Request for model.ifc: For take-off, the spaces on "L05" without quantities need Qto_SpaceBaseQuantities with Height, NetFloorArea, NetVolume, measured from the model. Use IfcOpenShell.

First a look at what the model holds.

```python
import ifcopenshell
import ifcopenshell.util.element
import ifcopenshell.util.unit

model = ifcopenshell.open("model.ifc")
print(model.schema)
for unit_type in ("LENGTHUNIT", "AREAUNIT", "VOLUMEUNIT"):
    print(unit_type, ifcopenshell.util.unit.calculate_unit_scale(model, unit_type))
storey = next(s for s in model.by_type("IfcBuildingStorey") if s.Name == "L05")
spaces = [e for e in ifcopenshell.util.element.get_decomposition(storey) if e.is_a("IfcSpace")]
for e in sorted(spaces, key=lambda e: e.id()):
    print(e.id(), e.is_a(), e.Name, list(ifcopenshell.util.element.get_psets(e, qtos_only=True)), sep=" | ")
```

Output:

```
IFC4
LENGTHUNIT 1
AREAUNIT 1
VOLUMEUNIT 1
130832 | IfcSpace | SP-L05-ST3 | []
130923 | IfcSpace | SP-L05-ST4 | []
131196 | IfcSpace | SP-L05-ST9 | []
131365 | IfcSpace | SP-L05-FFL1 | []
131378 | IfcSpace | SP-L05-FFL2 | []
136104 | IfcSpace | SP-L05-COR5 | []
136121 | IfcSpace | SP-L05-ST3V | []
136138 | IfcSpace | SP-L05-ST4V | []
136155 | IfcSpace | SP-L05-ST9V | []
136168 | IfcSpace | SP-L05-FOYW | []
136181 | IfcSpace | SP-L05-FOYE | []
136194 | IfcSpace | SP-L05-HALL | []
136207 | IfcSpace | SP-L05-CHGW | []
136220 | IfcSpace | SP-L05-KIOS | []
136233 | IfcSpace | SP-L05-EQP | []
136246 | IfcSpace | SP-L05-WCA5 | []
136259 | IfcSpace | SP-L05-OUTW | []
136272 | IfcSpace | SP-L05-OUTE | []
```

```python
import ifcopenshell
import ifcopenshell.api.pset
import ifcopenshell.geom
import ifcopenshell.util.element
import ifcopenshell.util.shape
import ifcopenshell.util.unit

model = ifcopenshell.open("model.ifc")
unit_scale = ifcopenshell.util.unit.calculate_unit_scale(model)
area_scale = ifcopenshell.util.unit.calculate_unit_scale(model, "AREAUNIT")
volume_scale = ifcopenshell.util.unit.calculate_unit_scale(model, "VOLUMEUNIT")
settings = ifcopenshell.geom.settings()

storey = next(s for s in model.by_type("IfcBuildingStorey") if s.Name == "L05")
spaces = [e for e in ifcopenshell.util.element.get_decomposition(storey) if e.is_a("IfcSpace")]

for e in sorted(spaces, key=lambda e: e.id()):
    if ifcopenshell.util.element.get_psets(e, qtos_only=True, should_inherit=False):
        continue
    # Geometry comes back in metres, in the element's own axes.
    shape = ifcopenshell.geom.create_shape(settings, e)
    values = {
        "Height": ifcopenshell.util.shape.get_z(shape.geometry) / unit_scale,
        "NetFloorArea": ifcopenshell.util.shape.get_footprint_area(shape.geometry) / area_scale,
        "NetVolume": ifcopenshell.util.shape.get_volume(shape.geometry) / volume_scale,
    }
    qto = ifcopenshell.api.pset.add_qto(model, product=e, name="Qto_SpaceBaseQuantities")
    ifcopenshell.api.pset.edit_qto(model, qto=qto, properties=values)
    print(e.id(), {k: round(v, 3) for k, v in values.items()})

model.write("model_edited.ifc")
```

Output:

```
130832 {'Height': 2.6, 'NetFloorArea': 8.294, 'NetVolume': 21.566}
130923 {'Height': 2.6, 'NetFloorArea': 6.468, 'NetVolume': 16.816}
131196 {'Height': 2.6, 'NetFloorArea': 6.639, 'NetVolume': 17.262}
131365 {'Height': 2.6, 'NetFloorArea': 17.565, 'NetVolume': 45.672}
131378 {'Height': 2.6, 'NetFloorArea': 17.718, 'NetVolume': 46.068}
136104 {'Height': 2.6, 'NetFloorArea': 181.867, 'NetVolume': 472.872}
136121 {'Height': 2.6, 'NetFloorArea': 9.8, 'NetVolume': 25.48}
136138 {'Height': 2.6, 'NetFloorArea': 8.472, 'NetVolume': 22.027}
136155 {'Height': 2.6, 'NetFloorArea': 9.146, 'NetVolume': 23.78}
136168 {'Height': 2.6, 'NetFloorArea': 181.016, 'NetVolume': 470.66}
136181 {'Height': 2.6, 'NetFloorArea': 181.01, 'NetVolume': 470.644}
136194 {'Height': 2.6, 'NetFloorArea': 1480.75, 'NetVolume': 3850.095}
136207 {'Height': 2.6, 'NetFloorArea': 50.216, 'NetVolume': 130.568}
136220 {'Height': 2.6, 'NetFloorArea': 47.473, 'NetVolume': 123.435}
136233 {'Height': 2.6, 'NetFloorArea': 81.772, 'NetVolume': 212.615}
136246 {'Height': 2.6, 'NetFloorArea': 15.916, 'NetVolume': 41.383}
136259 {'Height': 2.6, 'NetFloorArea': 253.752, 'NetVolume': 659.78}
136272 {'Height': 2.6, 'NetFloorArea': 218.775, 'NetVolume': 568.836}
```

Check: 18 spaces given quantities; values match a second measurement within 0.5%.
